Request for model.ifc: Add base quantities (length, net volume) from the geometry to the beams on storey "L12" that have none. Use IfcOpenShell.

First a look at what the model holds.

```python
import ifcopenshell
import ifcopenshell.util.element
import ifcopenshell.util.unit

model = ifcopenshell.open("model.ifc")
print(model.schema)
for unit_type in ("LENGTHUNIT", "AREAUNIT", "VOLUMEUNIT"):
    print(unit_type, ifcopenshell.util.unit.calculate_unit_scale(model, unit_type))
storey = next(s for s in model.by_type("IfcBuildingStorey") if s.Name == "L12")
beams = [e for e in ifcopenshell.util.element.get_decomposition(storey) if e.is_a("IfcBeam")]
for e in sorted(beams, key=lambda e: e.id()):
    print(e.id(), e.is_a(), e.Name, list(ifcopenshell.util.element.get_psets(e, qtos_only=True)), sep=" | ")
```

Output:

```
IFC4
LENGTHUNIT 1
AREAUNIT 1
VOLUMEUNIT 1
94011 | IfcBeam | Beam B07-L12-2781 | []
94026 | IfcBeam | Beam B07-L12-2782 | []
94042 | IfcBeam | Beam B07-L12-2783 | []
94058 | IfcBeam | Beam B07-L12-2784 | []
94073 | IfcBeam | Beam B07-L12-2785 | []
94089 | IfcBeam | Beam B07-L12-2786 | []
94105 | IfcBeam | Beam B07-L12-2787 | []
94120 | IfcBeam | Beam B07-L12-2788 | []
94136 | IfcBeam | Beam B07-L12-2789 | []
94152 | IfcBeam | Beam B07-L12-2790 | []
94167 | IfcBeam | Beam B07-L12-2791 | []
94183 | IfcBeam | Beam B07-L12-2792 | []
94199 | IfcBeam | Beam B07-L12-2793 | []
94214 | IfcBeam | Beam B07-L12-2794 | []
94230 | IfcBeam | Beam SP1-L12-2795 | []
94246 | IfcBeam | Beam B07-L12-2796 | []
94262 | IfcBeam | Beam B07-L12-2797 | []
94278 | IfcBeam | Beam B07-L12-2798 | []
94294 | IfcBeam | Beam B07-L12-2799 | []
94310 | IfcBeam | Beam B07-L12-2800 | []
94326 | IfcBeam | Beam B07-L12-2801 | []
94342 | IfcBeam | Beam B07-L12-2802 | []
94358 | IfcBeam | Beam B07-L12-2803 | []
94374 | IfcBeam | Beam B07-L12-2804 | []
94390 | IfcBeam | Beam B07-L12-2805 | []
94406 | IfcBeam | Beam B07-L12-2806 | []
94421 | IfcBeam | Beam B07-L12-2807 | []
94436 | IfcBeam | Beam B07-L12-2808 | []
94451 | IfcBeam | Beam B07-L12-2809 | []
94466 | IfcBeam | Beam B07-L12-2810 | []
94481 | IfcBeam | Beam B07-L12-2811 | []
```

```python
import ifcopenshell
import ifcopenshell.api.pset
import ifcopenshell.geom
import ifcopenshell.util.element
import ifcopenshell.util.shape
import ifcopenshell.util.unit

model = ifcopenshell.open("model.ifc")
unit_scale = ifcopenshell.util.unit.calculate_unit_scale(model)
volume_scale = ifcopenshell.util.unit.calculate_unit_scale(model, "VOLUMEUNIT")
settings = ifcopenshell.geom.settings()

storey = next(s for s in model.by_type("IfcBuildingStorey") if s.Name == "L12")
beams = [e for e in ifcopenshell.util.element.get_decomposition(storey) if e.is_a("IfcBeam")]

for e in sorted(beams, key=lambda e: e.id()):
    if ifcopenshell.util.element.get_psets(e, qtos_only=True, should_inherit=False):
        continue
    # Geometry comes back in metres, in the element's own axes.
    shape = ifcopenshell.geom.create_shape(settings, e)
    values = {
        "Length": ifcopenshell.util.shape.get_max_xyz(shape.geometry) / unit_scale,
        "NetVolume": ifcopenshell.util.shape.get_volume(shape.geometry) / volume_scale,
    }
    qto = ifcopenshell.api.pset.add_qto(model, product=e, name="Qto_BeamBaseQuantities")
    ifcopenshell.api.pset.edit_qto(model, qto=qto, properties=values)
    print(e.id(), {k: round(v, 3) for k, v in values.items()})

model.write("model_v2.ifc")
```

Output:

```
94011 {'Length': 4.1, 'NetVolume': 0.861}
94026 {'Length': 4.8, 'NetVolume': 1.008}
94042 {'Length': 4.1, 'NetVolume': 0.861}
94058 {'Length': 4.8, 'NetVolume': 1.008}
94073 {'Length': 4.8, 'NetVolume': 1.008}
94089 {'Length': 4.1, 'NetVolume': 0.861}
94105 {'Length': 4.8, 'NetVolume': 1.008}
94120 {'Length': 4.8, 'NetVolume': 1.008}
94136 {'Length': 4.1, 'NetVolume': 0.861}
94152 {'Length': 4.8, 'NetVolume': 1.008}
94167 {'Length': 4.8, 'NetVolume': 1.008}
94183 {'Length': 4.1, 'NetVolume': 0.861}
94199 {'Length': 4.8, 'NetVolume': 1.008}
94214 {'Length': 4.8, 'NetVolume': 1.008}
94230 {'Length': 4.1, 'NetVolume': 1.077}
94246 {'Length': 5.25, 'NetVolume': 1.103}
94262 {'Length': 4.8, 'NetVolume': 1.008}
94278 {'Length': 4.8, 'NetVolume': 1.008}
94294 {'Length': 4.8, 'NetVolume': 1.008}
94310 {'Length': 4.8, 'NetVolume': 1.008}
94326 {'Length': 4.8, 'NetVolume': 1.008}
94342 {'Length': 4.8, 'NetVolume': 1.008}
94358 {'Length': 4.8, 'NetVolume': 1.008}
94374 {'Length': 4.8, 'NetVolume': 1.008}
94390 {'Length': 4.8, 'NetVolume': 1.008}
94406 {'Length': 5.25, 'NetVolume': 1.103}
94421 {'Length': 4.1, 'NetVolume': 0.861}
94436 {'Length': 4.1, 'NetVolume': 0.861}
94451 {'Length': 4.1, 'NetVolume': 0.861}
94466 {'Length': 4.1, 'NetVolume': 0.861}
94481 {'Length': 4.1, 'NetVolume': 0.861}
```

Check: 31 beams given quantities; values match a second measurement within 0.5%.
